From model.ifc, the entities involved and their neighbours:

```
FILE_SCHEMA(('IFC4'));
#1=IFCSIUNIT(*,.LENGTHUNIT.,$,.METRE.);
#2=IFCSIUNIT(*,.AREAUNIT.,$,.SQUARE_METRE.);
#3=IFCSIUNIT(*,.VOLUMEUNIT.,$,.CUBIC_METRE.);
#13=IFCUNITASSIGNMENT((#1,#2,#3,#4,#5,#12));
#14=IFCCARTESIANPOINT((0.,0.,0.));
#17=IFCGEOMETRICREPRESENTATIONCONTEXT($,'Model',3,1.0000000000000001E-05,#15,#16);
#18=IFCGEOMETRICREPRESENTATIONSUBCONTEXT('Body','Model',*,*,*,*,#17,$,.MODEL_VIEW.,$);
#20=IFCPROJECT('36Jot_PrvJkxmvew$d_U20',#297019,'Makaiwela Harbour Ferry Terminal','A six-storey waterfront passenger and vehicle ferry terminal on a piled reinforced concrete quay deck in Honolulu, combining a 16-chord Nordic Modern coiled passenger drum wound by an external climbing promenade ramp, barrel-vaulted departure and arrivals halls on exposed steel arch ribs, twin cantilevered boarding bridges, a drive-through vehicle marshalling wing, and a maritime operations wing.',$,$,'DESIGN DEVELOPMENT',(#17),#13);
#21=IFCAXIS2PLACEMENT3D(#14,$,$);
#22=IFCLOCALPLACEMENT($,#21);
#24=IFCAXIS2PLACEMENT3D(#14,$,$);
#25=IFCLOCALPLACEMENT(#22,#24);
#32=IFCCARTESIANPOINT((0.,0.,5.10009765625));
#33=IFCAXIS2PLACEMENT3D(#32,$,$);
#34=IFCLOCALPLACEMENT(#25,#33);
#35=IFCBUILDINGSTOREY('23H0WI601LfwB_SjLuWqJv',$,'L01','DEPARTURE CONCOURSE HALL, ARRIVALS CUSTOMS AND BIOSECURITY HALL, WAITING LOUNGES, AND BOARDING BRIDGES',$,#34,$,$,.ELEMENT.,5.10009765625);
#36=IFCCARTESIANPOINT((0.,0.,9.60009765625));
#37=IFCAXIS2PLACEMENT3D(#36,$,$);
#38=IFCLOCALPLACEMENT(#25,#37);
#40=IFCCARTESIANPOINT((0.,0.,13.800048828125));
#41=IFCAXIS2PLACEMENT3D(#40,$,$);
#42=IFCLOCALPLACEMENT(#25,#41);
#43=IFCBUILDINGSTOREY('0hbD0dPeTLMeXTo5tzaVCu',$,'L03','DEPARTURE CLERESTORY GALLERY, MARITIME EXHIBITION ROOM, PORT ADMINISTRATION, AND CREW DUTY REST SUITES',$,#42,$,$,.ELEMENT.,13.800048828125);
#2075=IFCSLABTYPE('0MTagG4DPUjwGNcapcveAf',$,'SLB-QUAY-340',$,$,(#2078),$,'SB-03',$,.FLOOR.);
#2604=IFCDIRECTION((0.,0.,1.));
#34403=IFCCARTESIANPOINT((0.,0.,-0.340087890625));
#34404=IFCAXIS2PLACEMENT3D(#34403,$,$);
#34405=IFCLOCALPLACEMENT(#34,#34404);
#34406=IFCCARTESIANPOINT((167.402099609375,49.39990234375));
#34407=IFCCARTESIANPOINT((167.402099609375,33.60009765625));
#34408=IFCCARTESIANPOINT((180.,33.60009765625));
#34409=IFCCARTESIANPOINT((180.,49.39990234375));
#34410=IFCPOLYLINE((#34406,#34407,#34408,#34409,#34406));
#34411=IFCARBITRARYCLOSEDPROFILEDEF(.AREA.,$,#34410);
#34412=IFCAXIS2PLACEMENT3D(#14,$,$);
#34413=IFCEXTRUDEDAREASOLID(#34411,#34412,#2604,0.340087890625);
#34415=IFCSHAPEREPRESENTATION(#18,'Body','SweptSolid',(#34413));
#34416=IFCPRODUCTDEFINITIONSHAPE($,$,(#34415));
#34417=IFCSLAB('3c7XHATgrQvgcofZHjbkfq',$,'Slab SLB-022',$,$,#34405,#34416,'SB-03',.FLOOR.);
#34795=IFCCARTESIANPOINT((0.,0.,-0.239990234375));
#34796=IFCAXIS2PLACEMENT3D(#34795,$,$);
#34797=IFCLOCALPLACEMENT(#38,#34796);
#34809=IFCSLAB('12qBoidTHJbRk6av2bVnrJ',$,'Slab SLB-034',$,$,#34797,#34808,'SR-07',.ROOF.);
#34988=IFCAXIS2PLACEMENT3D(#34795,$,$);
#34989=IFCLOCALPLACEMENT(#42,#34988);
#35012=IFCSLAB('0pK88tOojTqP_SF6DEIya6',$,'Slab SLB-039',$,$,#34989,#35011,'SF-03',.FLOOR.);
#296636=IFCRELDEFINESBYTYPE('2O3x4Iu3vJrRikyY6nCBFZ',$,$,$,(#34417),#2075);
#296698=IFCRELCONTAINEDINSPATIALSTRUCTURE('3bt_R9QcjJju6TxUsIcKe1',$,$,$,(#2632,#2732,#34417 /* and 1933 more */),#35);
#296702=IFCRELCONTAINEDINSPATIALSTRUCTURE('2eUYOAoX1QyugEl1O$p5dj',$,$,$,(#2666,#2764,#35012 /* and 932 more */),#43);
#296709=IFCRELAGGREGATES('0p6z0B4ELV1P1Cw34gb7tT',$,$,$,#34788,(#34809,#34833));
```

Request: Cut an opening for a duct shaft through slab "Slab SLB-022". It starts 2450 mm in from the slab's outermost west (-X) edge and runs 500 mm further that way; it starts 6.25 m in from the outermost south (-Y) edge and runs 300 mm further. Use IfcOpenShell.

```python
import numpy as np
import ifcopenshell
import ifcopenshell.api.feature
import ifcopenshell.api.geometry
import ifcopenshell.api.root
import ifcopenshell.geom
import ifcopenshell.util.placement
import ifcopenshell.util.representation
import ifcopenshell.util.shape
import ifcopenshell.util.unit

model = ifcopenshell.open("model.ifc")
unit_scale = ifcopenshell.util.unit.calculate_unit_scale(model)
settings = ifcopenshell.geom.settings()


def volume(element):
    """Net volume in cubic metres, openings subtracted."""
    shape = ifcopenshell.geom.create_shape(settings, element)
    return ifcopenshell.util.shape.get_volume(shape.geometry)


slab = model.by_guid("3c7XHATgrQvgcofZHjbkfq")
before = volume(slab)

# Extent in the slab's own axes, in metres. The edges named are its -X and -Y sides.
slab_shape = ifcopenshell.geom.create_shape(settings, slab)
vertices = ifcopenshell.util.shape.get_vertices(slab_shape.geometry)
x_min, y_min, bottom = vertices.min(axis=0)
top = vertices[:, 2].max()

opening = ifcopenshell.api.root.create_entity(model, ifc_class="IfcOpeningElement", name="Duct shaft opening", predefined_type="OPENING")
context = ifcopenshell.util.representation.get_context(model, "Model", "Body", "MODEL_VIEW")
width, depth = 0.5, 0.3
outline = [(0.0, 0.0), (width, 0.0), (width, depth), (0.0, depth), (0.0, 0.0)]
# Overshoot both faces by 50 mm so the cut is clean.
shape = ifcopenshell.api.geometry.add_slab_representation(
    model, context=context, depth=top - bottom + 0.1, polyline=outline
)
ifcopenshell.api.geometry.assign_representation(model, product=opening, representation=shape)

matrix = ifcopenshell.util.placement.get_local_placement(slab.ObjectPlacement)
matrix[:, 3] = matrix @ np.append(np.array([x_min + 2.45, y_min + 6.25, bottom - 0.05]) / unit_scale, 1.0)
ifcopenshell.api.geometry.edit_object_placement(model, product=opening, matrix=matrix, is_si=False)
ifcopenshell.api.feature.add_feature(model, feature=opening, element=slab)

after = volume(slab)

print(f"slab volume {before:.3f} -> {after:.3f} m3")

model.write("model_updated.ifc")
```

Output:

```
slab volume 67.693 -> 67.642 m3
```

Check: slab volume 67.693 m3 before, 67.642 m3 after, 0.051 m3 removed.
